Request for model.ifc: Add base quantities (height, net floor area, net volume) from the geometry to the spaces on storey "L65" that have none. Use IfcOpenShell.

First a look at what the model holds.

```python
import ifcopenshell
import ifcopenshell.util.element
import ifcopenshell.util.unit

model = ifcopenshell.open("model.ifc")
print(model.schema)
for unit_type in ("LENGTHUNIT", "AREAUNIT", "VOLUMEUNIT"):
    print(unit_type, ifcopenshell.util.unit.calculate_unit_scale(model, unit_type))
storey = next(s for s in model.by_type("IfcBuildingStorey") if s.Name == "L65")
spaces = [e for e in ifcopenshell.util.element.get_decomposition(storey) if e.is_a("IfcSpace")]
for e in sorted(spaces, key=lambda e: e.id()):
    print(e.id(), e.is_a(), e.Name, list(ifcopenshell.util.element.get_psets(e, qtos_only=True)), sep=" | ")
```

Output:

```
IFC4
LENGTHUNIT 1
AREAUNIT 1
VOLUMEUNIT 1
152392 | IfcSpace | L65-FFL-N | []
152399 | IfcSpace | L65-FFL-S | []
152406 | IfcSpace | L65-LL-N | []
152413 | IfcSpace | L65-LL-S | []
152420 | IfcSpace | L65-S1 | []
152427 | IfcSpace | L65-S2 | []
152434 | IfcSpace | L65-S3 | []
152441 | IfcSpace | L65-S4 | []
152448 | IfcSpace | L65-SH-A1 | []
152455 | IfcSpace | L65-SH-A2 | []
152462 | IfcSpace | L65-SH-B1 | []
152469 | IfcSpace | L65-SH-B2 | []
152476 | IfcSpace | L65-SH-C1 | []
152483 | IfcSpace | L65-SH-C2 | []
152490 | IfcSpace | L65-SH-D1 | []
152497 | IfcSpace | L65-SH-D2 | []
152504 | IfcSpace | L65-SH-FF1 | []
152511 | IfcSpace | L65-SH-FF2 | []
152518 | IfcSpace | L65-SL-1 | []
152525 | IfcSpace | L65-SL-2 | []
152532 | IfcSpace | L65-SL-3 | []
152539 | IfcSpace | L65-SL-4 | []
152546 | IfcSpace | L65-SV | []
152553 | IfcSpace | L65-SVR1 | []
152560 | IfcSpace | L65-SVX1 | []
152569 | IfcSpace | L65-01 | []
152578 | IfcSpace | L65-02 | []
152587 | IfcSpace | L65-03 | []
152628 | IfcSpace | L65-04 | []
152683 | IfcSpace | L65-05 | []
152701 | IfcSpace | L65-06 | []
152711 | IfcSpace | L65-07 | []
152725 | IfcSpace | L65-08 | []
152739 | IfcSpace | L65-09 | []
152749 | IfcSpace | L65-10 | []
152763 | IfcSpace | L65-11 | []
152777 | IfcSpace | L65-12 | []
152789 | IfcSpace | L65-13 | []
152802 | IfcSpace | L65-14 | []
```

```python
import ifcopenshell
import ifcopenshell.api.pset
import ifcopenshell.geom
import ifcopenshell.util.element
import ifcopenshell.util.shape
import ifcopenshell.util.unit

model = ifcopenshell.open("model.ifc")
unit_scale = ifcopenshell.util.unit.calculate_unit_scale(model)
area_scale = ifcopenshell.util.unit.calculate_unit_scale(model, "AREAUNIT")
volume_scale = ifcopenshell.util.unit.calculate_unit_scale(model, "VOLUMEUNIT")
settings = ifcopenshell.geom.settings()

storey = next(s for s in model.by_type("IfcBuildingStorey") if s.Name == "L65")
spaces = [e for e in ifcopenshell.util.element.get_decomposition(storey) if e.is_a("IfcSpace")]

for e in sorted(spaces, key=lambda e: e.id()):
    if ifcopenshell.util.element.get_psets(e, qtos_only=True, should_inherit=False):
        continue
    # Geometry comes back in metres, in the element's own axes.
    shape = ifcopenshell.geom.create_shape(settings, e)
    values = {
        "Height": ifcopenshell.util.shape.get_z(shape.geometry) / unit_scale,
        "NetFloorArea": ifcopenshell.util.shape.get_footprint_area(shape.geometry) / area_scale,
        "NetVolume": ifcopenshell.util.shape.get_volume(shape.geometry) / volume_scale,
    }
    qto = ifcopenshell.api.pset.add_qto(model, product=e, name="Qto_SpaceBaseQuantities")
    ifcopenshell.api.pset.edit_qto(model, qto=qto, properties=values)
    print(e.id(), {k: round(v, 3) for k, v in values.items()})

model.write("model_edited.ifc")
```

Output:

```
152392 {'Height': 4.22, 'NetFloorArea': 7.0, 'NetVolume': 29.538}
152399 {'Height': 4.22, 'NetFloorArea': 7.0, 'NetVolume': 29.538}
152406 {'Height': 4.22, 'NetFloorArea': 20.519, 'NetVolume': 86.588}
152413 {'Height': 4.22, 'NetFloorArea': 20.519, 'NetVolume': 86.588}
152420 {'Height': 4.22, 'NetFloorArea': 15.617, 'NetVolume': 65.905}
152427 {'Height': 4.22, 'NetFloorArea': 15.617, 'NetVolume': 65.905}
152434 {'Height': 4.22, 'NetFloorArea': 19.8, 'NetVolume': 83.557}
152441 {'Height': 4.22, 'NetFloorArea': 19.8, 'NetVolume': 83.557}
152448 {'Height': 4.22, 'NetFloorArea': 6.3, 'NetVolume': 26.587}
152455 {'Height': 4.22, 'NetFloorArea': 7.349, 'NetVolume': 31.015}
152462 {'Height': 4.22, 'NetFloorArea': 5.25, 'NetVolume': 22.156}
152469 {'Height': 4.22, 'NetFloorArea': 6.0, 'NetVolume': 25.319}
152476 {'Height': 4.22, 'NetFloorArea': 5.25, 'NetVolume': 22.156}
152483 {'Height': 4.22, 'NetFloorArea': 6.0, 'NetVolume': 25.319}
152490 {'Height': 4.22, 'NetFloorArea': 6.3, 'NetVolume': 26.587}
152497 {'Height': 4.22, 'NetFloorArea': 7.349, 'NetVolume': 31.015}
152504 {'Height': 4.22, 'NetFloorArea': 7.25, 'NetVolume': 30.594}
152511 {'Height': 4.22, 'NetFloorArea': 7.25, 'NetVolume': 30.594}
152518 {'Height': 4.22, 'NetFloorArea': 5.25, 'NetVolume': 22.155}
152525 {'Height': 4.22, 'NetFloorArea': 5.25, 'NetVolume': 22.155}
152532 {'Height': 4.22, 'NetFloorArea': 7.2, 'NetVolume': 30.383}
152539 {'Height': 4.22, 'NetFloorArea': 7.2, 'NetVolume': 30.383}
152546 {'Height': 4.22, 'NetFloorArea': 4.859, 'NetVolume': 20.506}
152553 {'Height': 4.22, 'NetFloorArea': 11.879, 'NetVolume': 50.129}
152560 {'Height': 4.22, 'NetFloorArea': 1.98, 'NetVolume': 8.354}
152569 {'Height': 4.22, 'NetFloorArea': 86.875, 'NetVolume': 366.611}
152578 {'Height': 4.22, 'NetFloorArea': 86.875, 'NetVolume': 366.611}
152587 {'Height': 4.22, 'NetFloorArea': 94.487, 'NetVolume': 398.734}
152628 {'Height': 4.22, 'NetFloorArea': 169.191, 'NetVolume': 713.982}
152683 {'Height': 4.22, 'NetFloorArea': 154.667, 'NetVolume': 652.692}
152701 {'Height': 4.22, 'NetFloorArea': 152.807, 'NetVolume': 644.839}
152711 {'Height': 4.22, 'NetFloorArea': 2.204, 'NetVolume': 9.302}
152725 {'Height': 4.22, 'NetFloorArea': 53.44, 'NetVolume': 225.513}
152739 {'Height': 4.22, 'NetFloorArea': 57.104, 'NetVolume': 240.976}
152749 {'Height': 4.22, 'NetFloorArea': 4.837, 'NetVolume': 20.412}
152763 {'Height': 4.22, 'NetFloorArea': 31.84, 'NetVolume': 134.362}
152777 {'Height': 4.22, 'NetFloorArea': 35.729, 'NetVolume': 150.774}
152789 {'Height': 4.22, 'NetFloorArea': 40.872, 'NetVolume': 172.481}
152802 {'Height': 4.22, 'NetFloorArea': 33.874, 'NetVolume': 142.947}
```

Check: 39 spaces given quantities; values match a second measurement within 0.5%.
